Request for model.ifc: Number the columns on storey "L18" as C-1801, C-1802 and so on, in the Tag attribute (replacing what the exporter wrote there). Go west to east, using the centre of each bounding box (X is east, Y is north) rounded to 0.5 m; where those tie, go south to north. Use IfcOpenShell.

First a look at what the model holds.

```python
import ifcopenshell
import ifcopenshell.util.element
import ifcopenshell.util.placement

model = ifcopenshell.open("model.ifc")
print(model.schema)
storey = next(s for s in model.by_type("IfcBuildingStorey") if s.Name == "L18")
columns = [e for e in ifcopenshell.util.element.get_decomposition(storey) if e.is_a("IfcColumn")]
for e in sorted(columns, key=lambda e: e.id()):
    origin = ifcopenshell.util.placement.get_local_placement(e.ObjectPlacement)[:3, 3]
    print(e.id(), e.Tag, e.Name, origin.round(2) + 0.0, sep=" | ")
```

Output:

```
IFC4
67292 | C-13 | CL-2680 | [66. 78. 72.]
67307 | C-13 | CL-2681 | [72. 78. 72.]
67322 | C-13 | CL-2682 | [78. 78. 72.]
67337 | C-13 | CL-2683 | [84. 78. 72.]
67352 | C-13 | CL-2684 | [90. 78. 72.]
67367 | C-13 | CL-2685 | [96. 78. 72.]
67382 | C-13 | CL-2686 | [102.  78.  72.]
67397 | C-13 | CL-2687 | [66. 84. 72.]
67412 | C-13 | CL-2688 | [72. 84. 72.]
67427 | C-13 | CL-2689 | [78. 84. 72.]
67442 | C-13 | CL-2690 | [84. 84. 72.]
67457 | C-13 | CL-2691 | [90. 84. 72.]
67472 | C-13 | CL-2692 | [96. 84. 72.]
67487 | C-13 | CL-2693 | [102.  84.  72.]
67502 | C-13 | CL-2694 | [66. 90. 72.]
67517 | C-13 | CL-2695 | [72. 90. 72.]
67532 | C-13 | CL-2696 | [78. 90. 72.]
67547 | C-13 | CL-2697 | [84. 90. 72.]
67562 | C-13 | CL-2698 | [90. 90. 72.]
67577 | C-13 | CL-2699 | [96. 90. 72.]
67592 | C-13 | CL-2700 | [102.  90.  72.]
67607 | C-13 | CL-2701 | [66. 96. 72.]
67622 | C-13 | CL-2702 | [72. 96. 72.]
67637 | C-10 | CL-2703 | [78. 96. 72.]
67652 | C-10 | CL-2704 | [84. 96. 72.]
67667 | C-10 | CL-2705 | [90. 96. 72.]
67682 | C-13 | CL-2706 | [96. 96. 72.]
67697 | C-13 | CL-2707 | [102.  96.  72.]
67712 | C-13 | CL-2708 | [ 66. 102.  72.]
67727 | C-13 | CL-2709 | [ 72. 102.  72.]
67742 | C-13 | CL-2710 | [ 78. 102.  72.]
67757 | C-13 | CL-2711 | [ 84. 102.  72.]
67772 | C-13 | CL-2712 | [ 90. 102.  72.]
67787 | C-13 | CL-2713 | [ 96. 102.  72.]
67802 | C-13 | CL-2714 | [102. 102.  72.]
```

```python
import ifcopenshell
import ifcopenshell.geom
import ifcopenshell.util.element
import ifcopenshell.util.shape

model = ifcopenshell.open("model.ifc")
settings = ifcopenshell.geom.settings()
settings.set("use-world-coords", True)


def centre(element):
    shape = ifcopenshell.geom.create_shape(settings, element)
    return ifcopenshell.util.shape.get_bbox_centroid(shape.geometry)


storey = next(s for s in model.by_type("IfcBuildingStorey") if s.Name == "L18")
columns = [e for e in ifcopenshell.util.element.get_decomposition(storey) if e.is_a("IfcColumn")]

# Insertion points can sit at a corner or the storey origin, so sort by the geometry (in metres).
centres = {e: centre(e) for e in columns}
columns.sort(key=lambda e: (round(centres[e][0] / 0.5), centres[e][1]))

for i, e in enumerate(columns, start=1):
    number = f"C-18{i:02d}"
    e.Tag = number
    print(e.id(), number)

model.write("model_rev.ifc")
```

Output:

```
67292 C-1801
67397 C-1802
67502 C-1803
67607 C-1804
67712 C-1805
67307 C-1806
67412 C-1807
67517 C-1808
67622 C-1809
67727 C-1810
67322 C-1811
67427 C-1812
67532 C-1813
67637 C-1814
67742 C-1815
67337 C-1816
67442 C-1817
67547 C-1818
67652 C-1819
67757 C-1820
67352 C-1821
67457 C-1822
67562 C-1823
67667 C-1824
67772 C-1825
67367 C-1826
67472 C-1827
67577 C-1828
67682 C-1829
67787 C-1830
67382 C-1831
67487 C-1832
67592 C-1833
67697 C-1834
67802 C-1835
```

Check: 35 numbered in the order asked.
